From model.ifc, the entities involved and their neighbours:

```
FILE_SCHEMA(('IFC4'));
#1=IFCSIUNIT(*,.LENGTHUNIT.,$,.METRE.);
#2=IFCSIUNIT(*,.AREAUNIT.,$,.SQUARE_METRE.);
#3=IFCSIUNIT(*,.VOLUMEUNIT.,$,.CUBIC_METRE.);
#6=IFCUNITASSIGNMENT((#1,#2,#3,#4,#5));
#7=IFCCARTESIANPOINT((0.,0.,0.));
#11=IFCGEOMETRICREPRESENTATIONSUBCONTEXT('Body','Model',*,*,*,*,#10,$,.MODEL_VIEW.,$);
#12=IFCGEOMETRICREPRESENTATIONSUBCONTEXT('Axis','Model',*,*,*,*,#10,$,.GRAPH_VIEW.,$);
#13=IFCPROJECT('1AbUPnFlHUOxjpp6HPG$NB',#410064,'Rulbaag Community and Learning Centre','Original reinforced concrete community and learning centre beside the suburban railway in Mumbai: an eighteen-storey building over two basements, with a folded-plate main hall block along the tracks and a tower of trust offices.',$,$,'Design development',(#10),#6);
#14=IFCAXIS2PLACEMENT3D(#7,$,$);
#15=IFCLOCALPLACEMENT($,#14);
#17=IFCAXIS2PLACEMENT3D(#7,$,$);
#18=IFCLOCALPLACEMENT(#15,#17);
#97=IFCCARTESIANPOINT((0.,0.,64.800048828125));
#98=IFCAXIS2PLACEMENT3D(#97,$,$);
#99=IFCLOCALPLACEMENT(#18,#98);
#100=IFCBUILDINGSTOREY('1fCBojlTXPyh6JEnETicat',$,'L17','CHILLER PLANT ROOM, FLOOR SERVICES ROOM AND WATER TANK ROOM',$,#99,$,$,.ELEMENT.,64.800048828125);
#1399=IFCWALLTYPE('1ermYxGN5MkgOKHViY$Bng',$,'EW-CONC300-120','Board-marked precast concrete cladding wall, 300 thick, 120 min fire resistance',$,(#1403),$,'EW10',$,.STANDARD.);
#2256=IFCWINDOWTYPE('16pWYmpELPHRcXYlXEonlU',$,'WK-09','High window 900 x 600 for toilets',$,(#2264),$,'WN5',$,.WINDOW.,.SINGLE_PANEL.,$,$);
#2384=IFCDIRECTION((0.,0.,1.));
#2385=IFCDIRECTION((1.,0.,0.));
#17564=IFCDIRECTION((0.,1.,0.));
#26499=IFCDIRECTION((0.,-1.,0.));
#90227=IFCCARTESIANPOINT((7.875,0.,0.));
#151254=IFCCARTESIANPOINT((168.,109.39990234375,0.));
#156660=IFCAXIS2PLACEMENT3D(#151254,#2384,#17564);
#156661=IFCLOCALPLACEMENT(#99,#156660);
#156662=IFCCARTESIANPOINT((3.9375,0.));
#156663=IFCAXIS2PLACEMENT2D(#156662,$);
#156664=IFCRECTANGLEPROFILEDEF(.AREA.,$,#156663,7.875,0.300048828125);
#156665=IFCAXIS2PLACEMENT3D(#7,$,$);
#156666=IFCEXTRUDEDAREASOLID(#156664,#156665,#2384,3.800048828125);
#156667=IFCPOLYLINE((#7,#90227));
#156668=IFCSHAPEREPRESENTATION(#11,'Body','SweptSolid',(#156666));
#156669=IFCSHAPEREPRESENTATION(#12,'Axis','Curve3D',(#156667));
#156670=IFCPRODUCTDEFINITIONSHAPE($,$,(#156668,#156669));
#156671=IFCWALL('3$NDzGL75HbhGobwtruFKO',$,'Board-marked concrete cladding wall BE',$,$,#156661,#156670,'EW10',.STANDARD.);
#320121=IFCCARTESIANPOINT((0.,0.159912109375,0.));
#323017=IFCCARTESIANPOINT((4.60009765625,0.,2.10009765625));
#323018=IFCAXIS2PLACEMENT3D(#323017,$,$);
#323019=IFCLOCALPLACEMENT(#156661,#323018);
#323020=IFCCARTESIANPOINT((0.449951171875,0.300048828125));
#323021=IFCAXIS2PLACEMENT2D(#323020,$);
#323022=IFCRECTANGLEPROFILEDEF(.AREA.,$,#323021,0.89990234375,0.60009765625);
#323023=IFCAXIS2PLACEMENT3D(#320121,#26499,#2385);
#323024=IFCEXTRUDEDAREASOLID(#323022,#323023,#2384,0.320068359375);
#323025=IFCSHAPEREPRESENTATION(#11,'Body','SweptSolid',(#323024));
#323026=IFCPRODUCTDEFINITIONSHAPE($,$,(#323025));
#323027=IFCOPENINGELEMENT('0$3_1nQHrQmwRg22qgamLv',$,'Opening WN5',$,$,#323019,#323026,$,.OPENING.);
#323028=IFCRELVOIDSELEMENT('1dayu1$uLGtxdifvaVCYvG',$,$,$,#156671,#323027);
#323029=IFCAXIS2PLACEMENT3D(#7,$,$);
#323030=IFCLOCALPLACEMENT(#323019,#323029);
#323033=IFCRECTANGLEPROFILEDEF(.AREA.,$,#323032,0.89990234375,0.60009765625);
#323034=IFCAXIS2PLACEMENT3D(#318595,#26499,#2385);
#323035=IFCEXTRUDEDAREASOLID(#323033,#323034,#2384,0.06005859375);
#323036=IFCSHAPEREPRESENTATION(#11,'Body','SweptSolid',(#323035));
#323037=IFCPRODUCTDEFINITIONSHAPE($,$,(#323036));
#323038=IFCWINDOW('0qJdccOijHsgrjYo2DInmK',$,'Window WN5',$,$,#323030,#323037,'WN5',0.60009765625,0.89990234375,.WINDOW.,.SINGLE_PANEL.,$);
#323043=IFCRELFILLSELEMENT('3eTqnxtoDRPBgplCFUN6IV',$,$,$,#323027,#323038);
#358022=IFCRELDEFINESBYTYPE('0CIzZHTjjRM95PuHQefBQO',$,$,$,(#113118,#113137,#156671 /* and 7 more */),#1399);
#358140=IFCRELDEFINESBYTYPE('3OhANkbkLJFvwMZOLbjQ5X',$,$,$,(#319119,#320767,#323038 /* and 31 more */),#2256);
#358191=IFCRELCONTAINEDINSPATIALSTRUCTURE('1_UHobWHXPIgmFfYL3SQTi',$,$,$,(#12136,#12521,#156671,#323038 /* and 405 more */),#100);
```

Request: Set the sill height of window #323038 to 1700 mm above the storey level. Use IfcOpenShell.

```python
import numpy as np
import ifcopenshell
import ifcopenshell.api.geometry
import ifcopenshell.geom
import ifcopenshell.util.element
import ifcopenshell.util.placement
import ifcopenshell.util.shape
import ifcopenshell.util.unit

model = ifcopenshell.open("model.ifc")
unit_scale = ifcopenshell.util.unit.calculate_unit_scale(model)

window = model.by_guid("0qJdccOijHsgrjYo2DInmK")
opening = window.FillsVoids[0].RelatingOpeningElement
storey = ifcopenshell.util.element.get_container(window, ifc_class="IfcBuildingStorey")
level = ifcopenshell.util.placement.get_local_placement(storey.ObjectPlacement)[2, 3]

# The opening's origin need not be at the sill, so measure its lowest point.
shape = ifcopenshell.geom.create_shape(ifcopenshell.geom.settings(), opening)
bottom = ifcopenshell.util.shape.get_shape_bottom_elevation(shape, shape.geometry) / unit_scale
dz = level + 1.7 / unit_scale - bottom

shift = np.array([0.0, 0.0, dz])
# The window is placed relative to its opening, so it follows when the opening moves.
matrix = ifcopenshell.util.placement.get_local_placement(opening.ObjectPlacement)
matrix[:3, 3] += shift
ifcopenshell.api.geometry.edit_object_placement(
    model, product=opening, matrix=matrix, is_si=False, should_transform_children=True
)

print(f"moved by {dz * unit_scale:+.3f} m")

model.write("model_v2.ifc")
```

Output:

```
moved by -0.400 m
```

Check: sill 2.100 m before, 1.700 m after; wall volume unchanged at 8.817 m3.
